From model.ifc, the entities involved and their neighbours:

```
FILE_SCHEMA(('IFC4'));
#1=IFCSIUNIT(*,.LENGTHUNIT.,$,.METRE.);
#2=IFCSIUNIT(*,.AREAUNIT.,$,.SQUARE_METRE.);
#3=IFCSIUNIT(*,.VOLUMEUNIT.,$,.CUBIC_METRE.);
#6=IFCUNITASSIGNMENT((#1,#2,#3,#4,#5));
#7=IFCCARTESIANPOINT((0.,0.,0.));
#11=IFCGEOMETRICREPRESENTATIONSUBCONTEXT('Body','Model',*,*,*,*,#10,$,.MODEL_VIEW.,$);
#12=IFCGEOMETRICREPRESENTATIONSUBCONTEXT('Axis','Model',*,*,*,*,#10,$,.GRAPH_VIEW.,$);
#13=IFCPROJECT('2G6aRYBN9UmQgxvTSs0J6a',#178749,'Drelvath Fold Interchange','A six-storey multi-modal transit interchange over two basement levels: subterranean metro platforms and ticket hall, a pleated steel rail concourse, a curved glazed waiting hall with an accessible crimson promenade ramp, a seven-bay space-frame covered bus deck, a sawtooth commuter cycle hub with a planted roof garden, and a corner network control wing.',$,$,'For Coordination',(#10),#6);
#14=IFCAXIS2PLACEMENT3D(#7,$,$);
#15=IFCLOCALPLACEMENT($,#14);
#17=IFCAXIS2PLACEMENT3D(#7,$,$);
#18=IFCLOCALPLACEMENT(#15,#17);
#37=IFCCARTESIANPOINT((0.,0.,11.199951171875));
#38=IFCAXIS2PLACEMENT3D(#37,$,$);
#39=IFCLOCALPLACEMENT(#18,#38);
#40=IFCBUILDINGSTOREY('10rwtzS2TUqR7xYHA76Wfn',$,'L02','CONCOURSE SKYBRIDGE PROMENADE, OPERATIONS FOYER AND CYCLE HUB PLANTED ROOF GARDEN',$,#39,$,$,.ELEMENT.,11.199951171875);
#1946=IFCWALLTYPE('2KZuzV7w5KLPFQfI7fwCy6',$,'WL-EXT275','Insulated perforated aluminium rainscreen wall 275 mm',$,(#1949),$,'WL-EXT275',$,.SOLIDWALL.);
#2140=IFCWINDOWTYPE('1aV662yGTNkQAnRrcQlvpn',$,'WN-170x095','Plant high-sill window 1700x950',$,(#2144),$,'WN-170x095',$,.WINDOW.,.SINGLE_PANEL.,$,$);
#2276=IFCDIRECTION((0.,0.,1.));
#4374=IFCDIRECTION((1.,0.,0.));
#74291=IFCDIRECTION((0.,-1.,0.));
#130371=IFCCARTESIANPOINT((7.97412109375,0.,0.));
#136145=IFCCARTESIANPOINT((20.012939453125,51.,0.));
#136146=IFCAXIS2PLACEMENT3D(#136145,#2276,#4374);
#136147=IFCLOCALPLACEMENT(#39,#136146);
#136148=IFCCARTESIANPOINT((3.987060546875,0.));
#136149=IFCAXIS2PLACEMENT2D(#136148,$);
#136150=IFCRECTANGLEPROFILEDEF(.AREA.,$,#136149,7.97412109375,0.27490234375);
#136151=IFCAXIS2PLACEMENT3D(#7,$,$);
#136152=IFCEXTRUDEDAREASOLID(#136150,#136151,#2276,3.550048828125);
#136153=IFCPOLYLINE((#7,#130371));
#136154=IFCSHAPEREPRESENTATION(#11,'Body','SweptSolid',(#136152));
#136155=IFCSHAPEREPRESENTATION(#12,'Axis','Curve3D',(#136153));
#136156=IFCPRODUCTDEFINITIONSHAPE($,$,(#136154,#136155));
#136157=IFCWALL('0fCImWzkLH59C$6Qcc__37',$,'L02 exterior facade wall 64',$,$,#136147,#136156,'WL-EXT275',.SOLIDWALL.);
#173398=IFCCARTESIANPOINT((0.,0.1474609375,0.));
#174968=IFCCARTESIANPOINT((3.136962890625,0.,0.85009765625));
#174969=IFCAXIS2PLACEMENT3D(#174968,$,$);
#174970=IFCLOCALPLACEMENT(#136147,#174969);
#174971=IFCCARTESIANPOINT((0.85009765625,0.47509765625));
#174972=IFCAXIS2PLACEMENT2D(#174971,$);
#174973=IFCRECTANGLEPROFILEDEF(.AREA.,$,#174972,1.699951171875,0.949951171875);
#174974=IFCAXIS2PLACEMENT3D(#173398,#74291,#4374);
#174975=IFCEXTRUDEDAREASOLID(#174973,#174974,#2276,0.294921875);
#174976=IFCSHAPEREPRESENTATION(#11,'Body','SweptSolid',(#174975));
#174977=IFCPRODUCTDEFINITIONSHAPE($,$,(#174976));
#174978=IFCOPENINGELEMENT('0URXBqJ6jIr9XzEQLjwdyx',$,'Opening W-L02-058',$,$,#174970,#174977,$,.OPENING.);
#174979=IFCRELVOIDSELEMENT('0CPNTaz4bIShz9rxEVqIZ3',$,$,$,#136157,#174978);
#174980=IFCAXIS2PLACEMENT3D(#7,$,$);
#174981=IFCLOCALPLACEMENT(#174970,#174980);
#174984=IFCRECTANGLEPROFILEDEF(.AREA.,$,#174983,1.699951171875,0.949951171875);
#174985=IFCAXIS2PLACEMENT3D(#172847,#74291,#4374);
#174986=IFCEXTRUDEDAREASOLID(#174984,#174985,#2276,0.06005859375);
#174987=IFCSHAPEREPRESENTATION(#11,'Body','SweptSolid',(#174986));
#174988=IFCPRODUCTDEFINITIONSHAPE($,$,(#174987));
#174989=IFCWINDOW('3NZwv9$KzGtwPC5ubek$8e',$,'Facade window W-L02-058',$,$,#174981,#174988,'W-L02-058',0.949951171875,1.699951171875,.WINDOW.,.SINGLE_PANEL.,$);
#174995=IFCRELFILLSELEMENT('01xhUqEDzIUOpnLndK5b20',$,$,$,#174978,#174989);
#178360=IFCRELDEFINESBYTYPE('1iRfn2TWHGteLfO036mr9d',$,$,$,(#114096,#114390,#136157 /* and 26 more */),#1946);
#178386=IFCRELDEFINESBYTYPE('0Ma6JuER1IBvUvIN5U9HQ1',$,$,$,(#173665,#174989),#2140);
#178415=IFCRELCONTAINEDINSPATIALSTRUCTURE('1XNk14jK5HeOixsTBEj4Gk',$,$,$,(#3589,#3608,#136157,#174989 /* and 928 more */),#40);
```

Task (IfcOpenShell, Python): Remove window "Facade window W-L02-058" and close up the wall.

```python
import ifcopenshell
import ifcopenshell.api.feature
import ifcopenshell.api.root
import ifcopenshell.geom
import ifcopenshell.util.shape

model = ifcopenshell.open("model.ifc")
settings = ifcopenshell.geom.settings()


def volume(element):
    """Net volume in cubic metres, openings subtracted."""
    shape = ifcopenshell.geom.create_shape(settings, element)
    return ifcopenshell.util.shape.get_volume(shape.geometry)


window = model.by_guid("3NZwv9$KzGtwPC5ubek$8e")
opening = window.FillsVoids[0].RelatingOpeningElement
wall = opening.VoidsElements[0].RelatingBuildingElement
before = volume(wall)

ifcopenshell.api.root.remove_product(model, product=window)
ifcopenshell.api.feature.remove_feature(model, feature=opening)

after = volume(wall)

print(f"wall volume {before:.3f} -> {after:.3f} m3")

model.write("model_edited.ifc")
```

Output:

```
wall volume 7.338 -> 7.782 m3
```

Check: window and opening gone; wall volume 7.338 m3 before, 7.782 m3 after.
